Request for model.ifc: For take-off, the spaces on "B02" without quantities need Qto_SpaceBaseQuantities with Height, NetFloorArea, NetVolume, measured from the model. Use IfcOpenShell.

First a look at what the model holds.

```python
import ifcopenshell
import ifcopenshell.util.element
import ifcopenshell.util.unit

model = ifcopenshell.open("model.ifc")
print(model.schema)
for unit_type in ("LENGTHUNIT", "AREAUNIT", "VOLUMEUNIT"):
    print(unit_type, ifcopenshell.util.unit.calculate_unit_scale(model, unit_type))
storey = next(s for s in model.by_type("IfcBuildingStorey") if s.Name == "B02")
spaces = [e for e in ifcopenshell.util.element.get_decomposition(storey) if e.is_a("IfcSpace")]
for e in sorted(spaces, key=lambda e: e.id()):
    print(e.id(), e.is_a(), e.Name, list(ifcopenshell.util.element.get_psets(e, qtos_only=True)), sep=" | ")
```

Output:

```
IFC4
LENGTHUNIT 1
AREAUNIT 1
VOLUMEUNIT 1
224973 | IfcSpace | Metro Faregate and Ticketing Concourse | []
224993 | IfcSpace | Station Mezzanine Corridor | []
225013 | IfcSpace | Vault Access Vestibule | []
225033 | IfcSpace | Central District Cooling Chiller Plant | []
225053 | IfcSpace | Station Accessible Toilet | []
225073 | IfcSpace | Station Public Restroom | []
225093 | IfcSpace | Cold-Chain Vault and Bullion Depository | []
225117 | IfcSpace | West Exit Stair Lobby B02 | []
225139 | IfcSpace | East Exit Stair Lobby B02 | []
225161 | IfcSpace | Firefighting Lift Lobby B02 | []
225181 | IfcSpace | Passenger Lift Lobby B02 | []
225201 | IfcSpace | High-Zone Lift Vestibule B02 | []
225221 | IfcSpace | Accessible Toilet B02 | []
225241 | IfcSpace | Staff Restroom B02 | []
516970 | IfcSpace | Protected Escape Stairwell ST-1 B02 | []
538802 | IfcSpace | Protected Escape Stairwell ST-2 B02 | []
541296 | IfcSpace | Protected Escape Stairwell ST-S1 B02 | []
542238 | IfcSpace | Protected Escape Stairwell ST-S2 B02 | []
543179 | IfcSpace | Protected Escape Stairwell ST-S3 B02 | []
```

```python
import ifcopenshell
import ifcopenshell.api.pset
import ifcopenshell.geom
import ifcopenshell.util.element
import ifcopenshell.util.shape
import ifcopenshell.util.unit

model = ifcopenshell.open("model.ifc")
unit_scale = ifcopenshell.util.unit.calculate_unit_scale(model)
area_scale = ifcopenshell.util.unit.calculate_unit_scale(model, "AREAUNIT")
volume_scale = ifcopenshell.util.unit.calculate_unit_scale(model, "VOLUMEUNIT")
settings = ifcopenshell.geom.settings()

storey = next(s for s in model.by_type("IfcBuildingStorey") if s.Name == "B02")
spaces = [e for e in ifcopenshell.util.element.get_decomposition(storey) if e.is_a("IfcSpace")]

for e in sorted(spaces, key=lambda e: e.id()):
    if ifcopenshell.util.element.get_psets(e, qtos_only=True, should_inherit=False):
        continue
    # Geometry comes back in metres, in the element's own axes.
    shape = ifcopenshell.geom.create_shape(settings, e)
    values = {
        "Height": ifcopenshell.util.shape.get_z(shape.geometry) / unit_scale,
        "NetFloorArea": ifcopenshell.util.shape.get_footprint_area(shape.geometry) / area_scale,
        "NetVolume": ifcopenshell.util.shape.get_volume(shape.geometry) / volume_scale,
    }
    qto = ifcopenshell.api.pset.add_qto(model, product=e, name="Qto_SpaceBaseQuantities")
    ifcopenshell.api.pset.edit_qto(model, qto=qto, properties=values)
    print(e.id(), {k: round(v, 3) for k, v in values.items()})

model.write("model_edited.ifc")
```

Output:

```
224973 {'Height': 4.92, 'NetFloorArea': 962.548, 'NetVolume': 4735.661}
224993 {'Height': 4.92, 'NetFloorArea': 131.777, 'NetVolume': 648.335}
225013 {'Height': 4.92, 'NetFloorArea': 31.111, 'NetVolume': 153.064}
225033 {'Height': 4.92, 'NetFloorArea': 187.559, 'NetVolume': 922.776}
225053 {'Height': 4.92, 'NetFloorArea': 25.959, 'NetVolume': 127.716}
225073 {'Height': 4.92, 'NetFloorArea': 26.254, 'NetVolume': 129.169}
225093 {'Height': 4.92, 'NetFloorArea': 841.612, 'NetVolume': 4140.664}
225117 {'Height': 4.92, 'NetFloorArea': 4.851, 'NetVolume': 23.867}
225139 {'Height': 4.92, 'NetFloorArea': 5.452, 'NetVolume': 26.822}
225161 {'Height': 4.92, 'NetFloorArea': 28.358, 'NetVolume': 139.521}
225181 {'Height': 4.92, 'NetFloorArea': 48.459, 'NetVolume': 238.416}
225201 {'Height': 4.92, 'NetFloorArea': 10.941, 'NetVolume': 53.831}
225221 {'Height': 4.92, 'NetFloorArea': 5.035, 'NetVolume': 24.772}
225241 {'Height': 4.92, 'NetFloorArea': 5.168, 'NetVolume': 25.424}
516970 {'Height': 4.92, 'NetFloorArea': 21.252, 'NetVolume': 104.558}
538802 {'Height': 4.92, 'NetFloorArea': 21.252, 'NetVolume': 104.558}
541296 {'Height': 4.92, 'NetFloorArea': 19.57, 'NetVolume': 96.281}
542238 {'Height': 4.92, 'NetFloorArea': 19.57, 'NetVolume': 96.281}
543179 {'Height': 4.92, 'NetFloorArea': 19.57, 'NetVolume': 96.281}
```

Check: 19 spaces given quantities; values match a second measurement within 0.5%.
